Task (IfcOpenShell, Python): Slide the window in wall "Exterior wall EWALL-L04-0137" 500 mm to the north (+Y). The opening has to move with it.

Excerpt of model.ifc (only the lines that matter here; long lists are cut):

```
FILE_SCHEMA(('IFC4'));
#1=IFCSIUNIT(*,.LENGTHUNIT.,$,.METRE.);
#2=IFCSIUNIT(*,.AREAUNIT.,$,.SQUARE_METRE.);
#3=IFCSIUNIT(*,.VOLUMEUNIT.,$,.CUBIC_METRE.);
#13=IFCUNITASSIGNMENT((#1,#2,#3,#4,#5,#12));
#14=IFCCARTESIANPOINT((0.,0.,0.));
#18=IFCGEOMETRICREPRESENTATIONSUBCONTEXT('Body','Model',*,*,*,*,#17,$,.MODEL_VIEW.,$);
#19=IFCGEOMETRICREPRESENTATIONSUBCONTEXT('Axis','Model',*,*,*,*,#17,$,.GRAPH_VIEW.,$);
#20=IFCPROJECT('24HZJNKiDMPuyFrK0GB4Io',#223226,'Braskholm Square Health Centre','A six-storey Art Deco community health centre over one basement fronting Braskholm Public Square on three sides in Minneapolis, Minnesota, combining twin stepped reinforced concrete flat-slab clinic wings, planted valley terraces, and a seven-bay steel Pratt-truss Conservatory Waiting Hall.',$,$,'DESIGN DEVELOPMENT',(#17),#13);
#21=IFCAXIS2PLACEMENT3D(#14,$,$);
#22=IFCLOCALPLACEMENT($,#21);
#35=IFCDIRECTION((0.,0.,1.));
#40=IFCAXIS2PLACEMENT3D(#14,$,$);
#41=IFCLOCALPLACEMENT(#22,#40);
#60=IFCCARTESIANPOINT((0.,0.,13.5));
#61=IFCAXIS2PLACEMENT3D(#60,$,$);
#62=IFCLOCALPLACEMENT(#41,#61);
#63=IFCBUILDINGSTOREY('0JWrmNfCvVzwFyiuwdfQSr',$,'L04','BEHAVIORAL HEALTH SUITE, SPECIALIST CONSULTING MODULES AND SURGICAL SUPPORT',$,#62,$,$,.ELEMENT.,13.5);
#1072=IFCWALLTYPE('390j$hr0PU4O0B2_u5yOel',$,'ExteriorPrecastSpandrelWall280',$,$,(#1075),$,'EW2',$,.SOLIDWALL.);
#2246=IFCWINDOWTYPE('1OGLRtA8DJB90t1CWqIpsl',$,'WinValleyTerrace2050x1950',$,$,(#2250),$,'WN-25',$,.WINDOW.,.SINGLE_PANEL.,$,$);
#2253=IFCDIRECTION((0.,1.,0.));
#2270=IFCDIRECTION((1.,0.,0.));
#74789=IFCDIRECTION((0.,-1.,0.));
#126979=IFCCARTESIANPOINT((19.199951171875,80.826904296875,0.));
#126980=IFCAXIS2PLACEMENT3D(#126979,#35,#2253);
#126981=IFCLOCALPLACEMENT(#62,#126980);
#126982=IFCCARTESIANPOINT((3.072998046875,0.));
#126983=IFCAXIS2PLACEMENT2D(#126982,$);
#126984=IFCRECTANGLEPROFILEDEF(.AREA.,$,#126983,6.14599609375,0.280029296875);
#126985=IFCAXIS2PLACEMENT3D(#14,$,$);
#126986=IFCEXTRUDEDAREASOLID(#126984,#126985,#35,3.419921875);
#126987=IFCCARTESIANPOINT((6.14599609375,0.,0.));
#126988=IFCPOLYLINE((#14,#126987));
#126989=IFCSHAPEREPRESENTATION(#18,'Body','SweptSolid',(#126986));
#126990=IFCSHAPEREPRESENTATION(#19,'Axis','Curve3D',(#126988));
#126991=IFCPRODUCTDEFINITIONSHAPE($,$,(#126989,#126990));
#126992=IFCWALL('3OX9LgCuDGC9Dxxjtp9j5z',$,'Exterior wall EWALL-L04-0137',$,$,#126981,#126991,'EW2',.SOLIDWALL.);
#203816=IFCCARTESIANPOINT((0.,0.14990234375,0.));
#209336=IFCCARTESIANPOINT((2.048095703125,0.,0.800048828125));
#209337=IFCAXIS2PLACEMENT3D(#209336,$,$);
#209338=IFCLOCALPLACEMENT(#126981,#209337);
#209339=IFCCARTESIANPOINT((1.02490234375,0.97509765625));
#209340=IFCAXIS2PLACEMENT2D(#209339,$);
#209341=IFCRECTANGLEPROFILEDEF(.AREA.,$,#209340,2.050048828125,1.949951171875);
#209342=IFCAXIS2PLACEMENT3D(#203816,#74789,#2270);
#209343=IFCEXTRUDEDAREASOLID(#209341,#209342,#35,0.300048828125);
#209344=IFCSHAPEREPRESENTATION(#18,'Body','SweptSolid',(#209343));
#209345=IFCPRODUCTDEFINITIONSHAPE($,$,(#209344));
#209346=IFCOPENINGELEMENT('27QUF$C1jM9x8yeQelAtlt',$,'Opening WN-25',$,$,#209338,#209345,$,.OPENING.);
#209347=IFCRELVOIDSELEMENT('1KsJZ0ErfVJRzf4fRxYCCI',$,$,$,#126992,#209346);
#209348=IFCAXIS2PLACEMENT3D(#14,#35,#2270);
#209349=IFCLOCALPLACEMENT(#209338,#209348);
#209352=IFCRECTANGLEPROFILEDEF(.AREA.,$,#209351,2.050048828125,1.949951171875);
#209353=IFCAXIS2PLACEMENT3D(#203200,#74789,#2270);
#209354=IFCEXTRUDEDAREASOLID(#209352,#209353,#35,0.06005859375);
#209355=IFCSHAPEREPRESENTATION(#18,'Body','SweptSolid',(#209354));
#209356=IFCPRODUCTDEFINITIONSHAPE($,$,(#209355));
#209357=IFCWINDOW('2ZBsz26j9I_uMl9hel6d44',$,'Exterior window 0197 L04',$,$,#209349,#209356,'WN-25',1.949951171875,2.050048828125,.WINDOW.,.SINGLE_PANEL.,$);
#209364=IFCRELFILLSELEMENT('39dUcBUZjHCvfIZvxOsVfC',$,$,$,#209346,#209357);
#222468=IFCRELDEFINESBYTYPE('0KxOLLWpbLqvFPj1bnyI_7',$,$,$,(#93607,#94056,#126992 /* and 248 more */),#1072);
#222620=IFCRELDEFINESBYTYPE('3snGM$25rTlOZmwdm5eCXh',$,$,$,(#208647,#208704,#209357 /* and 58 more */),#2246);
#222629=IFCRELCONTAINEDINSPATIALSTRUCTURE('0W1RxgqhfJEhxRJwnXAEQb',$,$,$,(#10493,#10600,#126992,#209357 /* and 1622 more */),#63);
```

```python
import ifcopenshell
import ifcopenshell.api.geometry
import ifcopenshell.util.placement

model = ifcopenshell.open("model.ifc")

window = model.by_guid("2ZBsz26j9I_uMl9hel6d44")
opening = window.FillsVoids[0].RelatingOpeningElement
wall = opening.VoidsElements[0].RelatingBuildingElement

wall_matrix = ifcopenshell.util.placement.get_local_placement(wall.ObjectPlacement)
shift = wall_matrix[:3, 0] * 0.5
before = ifcopenshell.util.placement.get_local_placement(window.ObjectPlacement)[:3, 3].copy()

# The window is placed relative to its opening, so it follows when the opening moves.
matrix = ifcopenshell.util.placement.get_local_placement(opening.ObjectPlacement)
matrix[:3, 3] += shift
ifcopenshell.api.geometry.edit_object_placement(
    model, product=opening, matrix=matrix, is_si=False, should_transform_children=True
)

after = ifcopenshell.util.placement.get_local_placement(window.ObjectPlacement)[:3, 3]
print("window moved by", (after - before).round(3) + 0.0)

model.write("model-out.ifc")
```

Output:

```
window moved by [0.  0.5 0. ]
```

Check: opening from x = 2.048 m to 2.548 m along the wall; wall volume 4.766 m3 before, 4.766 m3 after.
